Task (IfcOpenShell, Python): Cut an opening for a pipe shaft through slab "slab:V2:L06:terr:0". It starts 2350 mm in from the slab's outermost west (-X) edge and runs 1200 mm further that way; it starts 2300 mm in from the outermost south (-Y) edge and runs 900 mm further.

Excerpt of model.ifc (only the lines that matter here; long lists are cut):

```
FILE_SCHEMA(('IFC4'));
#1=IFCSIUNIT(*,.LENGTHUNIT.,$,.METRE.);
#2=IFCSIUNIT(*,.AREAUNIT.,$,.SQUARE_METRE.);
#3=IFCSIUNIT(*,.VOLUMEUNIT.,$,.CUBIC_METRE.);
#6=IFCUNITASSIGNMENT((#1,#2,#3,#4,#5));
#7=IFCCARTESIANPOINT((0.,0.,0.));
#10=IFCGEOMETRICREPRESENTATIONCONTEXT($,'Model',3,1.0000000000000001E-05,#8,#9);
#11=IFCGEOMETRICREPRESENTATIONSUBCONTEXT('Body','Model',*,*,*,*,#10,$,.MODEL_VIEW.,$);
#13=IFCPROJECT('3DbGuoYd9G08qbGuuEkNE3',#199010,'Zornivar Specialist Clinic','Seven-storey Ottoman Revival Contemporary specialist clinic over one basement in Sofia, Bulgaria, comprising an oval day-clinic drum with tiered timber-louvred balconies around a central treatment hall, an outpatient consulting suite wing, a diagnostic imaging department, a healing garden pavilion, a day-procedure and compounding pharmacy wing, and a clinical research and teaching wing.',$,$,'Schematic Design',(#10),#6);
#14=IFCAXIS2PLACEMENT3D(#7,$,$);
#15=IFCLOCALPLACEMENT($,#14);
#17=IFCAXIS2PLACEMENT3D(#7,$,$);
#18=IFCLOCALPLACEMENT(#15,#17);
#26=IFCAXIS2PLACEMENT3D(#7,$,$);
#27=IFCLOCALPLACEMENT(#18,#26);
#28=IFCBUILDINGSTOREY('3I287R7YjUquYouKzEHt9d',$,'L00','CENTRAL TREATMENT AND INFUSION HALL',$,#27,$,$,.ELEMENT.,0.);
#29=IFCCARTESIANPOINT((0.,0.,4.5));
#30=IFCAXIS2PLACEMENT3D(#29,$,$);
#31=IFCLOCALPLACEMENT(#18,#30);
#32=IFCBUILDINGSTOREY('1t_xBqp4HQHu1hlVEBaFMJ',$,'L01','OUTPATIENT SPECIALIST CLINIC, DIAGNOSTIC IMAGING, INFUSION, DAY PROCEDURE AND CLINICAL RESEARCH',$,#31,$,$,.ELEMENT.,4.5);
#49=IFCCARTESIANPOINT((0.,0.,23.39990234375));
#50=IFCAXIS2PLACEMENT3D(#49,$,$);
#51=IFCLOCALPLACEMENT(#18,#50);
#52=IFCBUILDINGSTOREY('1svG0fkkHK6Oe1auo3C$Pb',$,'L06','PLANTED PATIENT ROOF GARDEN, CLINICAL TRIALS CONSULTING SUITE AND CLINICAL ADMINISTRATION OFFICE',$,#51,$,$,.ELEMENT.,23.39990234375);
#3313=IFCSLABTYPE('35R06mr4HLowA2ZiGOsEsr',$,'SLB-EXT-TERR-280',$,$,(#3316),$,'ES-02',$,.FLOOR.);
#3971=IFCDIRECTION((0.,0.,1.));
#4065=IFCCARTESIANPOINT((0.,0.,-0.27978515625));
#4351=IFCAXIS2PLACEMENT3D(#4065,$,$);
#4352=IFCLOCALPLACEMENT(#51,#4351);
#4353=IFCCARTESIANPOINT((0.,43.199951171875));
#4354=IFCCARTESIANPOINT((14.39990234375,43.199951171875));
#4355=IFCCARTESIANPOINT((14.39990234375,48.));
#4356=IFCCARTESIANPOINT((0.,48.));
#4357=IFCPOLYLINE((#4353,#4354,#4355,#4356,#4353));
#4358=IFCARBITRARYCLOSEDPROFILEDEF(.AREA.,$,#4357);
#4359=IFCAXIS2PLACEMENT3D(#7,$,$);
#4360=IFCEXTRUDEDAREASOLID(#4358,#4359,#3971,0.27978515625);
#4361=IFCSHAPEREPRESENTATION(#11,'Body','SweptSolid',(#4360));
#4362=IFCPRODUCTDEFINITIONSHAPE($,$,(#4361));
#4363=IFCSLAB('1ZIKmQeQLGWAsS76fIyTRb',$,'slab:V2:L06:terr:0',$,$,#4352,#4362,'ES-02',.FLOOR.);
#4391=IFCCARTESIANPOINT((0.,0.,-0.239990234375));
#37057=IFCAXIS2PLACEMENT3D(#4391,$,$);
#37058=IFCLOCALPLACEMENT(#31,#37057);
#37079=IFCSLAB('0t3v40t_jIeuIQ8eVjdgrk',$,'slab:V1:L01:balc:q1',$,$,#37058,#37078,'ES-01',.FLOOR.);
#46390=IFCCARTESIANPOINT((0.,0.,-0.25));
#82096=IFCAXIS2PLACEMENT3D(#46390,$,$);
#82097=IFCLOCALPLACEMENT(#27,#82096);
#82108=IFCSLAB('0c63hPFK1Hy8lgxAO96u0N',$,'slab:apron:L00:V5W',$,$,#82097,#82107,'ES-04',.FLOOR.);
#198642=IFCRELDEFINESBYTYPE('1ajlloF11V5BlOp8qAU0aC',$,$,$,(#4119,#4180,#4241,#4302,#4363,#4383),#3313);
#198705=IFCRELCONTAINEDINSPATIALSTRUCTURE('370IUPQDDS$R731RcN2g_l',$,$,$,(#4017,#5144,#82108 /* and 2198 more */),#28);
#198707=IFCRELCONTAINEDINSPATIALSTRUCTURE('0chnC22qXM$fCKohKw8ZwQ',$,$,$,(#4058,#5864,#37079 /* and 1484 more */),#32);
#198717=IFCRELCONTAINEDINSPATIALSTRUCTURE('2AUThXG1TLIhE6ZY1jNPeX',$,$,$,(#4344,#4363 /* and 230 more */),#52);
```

```python
import numpy as np
import ifcopenshell
import ifcopenshell.api.feature
import ifcopenshell.api.geometry
import ifcopenshell.api.root
import ifcopenshell.geom
import ifcopenshell.util.placement
import ifcopenshell.util.representation
import ifcopenshell.util.shape
import ifcopenshell.util.unit

model = ifcopenshell.open("model.ifc")
unit_scale = ifcopenshell.util.unit.calculate_unit_scale(model)
settings = ifcopenshell.geom.settings()


def volume(element):
    """Net volume in cubic metres, openings subtracted."""
    shape = ifcopenshell.geom.create_shape(settings, element)
    return ifcopenshell.util.shape.get_volume(shape.geometry)


slab = model.by_id(4363)
before = volume(slab)

# Extent in the slab's own axes, in metres. The edges named are its -X and -Y sides.
slab_shape = ifcopenshell.geom.create_shape(settings, slab)
vertices = ifcopenshell.util.shape.get_vertices(slab_shape.geometry)
x_min, y_min, bottom = vertices.min(axis=0)
top = vertices[:, 2].max()

opening = ifcopenshell.api.root.create_entity(model, ifc_class="IfcOpeningElement", name="Pipe shaft opening", predefined_type="OPENING")
context = ifcopenshell.util.representation.get_context(model, "Model", "Body", "MODEL_VIEW")
width, depth = 1.2, 0.9
outline = [(0.0, 0.0), (width, 0.0), (width, depth), (0.0, depth), (0.0, 0.0)]
# Overshoot both faces by 50 mm so the cut is clean.
shape = ifcopenshell.api.geometry.add_slab_representation(
    model, context=context, depth=top - bottom + 0.1, polyline=outline
)
ifcopenshell.api.geometry.assign_representation(model, product=opening, representation=shape)

matrix = ifcopenshell.util.placement.get_local_placement(slab.ObjectPlacement)
matrix[:, 3] = matrix @ np.append(np.array([x_min + 2.35, y_min + 2.3, bottom - 0.05]) / unit_scale, 1.0)
ifcopenshell.api.geometry.edit_object_placement(model, product=opening, matrix=matrix, is_si=False)
ifcopenshell.api.feature.add_feature(model, feature=opening, element=slab)

after = volume(slab)

print(f"slab volume {before:.3f} -> {after:.3f} m3")

model.write("model_edited.ifc")
```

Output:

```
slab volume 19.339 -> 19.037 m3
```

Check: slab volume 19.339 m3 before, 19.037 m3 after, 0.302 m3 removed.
